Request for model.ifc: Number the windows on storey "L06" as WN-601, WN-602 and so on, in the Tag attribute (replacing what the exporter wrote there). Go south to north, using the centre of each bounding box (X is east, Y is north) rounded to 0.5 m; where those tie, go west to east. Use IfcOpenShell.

First a look at what the model holds.

```python
import ifcopenshell
import ifcopenshell.util.element
import ifcopenshell.util.placement

model = ifcopenshell.open("model.ifc")
print(model.schema)
storey = next(s for s in model.by_type("IfcBuildingStorey") if s.Name == "L06")
windows = [e for e in ifcopenshell.util.element.get_decomposition(storey) if e.is_a("IfcWindow")]
for e in sorted(windows, key=lambda e: e.id()):
    origin = ifcopenshell.util.placement.get_local_placement(e.ObjectPlacement)[:3, 3]
    print(e.id(), e.Tag, e.Name, origin.round(2) + 0.0, sep=" | ")
```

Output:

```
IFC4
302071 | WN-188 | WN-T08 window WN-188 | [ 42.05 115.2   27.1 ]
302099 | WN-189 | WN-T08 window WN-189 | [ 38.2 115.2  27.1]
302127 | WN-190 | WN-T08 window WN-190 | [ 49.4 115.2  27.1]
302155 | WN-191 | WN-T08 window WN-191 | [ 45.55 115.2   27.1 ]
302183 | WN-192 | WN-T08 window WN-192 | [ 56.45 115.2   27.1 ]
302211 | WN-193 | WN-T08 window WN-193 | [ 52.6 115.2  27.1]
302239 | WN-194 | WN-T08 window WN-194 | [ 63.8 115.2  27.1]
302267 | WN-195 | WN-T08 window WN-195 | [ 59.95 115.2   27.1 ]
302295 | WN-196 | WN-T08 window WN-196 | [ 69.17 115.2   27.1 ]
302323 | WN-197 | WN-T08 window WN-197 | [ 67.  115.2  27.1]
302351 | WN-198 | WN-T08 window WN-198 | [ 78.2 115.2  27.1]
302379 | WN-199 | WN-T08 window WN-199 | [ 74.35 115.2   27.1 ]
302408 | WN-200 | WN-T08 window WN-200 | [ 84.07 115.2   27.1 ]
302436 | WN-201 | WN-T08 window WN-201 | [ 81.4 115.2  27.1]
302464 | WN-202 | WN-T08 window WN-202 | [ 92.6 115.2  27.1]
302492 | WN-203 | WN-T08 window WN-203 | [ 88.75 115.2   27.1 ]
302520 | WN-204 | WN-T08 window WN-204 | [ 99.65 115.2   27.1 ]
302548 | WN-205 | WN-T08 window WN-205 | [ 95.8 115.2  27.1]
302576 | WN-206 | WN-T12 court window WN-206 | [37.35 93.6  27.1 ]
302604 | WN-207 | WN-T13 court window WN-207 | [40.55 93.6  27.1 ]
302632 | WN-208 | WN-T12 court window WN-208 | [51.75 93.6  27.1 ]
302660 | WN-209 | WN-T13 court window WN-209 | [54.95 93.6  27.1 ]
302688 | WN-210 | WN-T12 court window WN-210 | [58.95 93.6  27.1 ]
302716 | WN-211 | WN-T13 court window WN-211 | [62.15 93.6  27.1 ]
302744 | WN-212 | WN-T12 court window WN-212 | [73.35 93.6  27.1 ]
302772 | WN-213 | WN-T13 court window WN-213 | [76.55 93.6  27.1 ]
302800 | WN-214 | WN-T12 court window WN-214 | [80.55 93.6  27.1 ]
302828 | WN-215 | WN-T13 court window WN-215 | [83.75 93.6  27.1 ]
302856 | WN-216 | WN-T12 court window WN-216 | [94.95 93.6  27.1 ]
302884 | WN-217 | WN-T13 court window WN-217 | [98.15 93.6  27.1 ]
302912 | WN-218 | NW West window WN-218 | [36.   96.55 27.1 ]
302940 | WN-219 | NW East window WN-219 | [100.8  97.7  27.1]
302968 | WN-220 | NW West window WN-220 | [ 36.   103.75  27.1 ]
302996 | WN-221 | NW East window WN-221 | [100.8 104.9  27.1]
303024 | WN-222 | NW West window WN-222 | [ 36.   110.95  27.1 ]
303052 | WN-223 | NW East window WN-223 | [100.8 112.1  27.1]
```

```python
import ifcopenshell
import ifcopenshell.geom
import ifcopenshell.util.element
import ifcopenshell.util.shape

model = ifcopenshell.open("model.ifc")
settings = ifcopenshell.geom.settings()
settings.set("use-world-coords", True)


def centre(element):
    shape = ifcopenshell.geom.create_shape(settings, element)
    return ifcopenshell.util.shape.get_bbox_centroid(shape.geometry)


storey = next(s for s in model.by_type("IfcBuildingStorey") if s.Name == "L06")
windows = [e for e in ifcopenshell.util.element.get_decomposition(storey) if e.is_a("IfcWindow")]

# Insertion points can sit at a corner or the storey origin, so sort by the geometry (in metres).
centres = {e: centre(e) for e in windows}
windows.sort(key=lambda e: (round(centres[e][1] / 0.5), centres[e][0]))

for i, e in enumerate(windows, start=1):
    number = f"WN-6{i:02d}"
    e.Tag = number
    print(e.id(), number)

model.write("model_v2.ifc")
```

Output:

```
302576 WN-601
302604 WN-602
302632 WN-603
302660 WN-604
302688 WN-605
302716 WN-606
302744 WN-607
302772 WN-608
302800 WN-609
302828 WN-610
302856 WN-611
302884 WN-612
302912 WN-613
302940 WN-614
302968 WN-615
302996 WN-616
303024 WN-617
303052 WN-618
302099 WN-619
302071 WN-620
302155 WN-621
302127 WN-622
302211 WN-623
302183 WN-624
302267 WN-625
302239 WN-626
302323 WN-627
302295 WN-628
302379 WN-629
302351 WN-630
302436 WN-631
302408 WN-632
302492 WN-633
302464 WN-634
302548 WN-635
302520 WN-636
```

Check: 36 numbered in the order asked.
